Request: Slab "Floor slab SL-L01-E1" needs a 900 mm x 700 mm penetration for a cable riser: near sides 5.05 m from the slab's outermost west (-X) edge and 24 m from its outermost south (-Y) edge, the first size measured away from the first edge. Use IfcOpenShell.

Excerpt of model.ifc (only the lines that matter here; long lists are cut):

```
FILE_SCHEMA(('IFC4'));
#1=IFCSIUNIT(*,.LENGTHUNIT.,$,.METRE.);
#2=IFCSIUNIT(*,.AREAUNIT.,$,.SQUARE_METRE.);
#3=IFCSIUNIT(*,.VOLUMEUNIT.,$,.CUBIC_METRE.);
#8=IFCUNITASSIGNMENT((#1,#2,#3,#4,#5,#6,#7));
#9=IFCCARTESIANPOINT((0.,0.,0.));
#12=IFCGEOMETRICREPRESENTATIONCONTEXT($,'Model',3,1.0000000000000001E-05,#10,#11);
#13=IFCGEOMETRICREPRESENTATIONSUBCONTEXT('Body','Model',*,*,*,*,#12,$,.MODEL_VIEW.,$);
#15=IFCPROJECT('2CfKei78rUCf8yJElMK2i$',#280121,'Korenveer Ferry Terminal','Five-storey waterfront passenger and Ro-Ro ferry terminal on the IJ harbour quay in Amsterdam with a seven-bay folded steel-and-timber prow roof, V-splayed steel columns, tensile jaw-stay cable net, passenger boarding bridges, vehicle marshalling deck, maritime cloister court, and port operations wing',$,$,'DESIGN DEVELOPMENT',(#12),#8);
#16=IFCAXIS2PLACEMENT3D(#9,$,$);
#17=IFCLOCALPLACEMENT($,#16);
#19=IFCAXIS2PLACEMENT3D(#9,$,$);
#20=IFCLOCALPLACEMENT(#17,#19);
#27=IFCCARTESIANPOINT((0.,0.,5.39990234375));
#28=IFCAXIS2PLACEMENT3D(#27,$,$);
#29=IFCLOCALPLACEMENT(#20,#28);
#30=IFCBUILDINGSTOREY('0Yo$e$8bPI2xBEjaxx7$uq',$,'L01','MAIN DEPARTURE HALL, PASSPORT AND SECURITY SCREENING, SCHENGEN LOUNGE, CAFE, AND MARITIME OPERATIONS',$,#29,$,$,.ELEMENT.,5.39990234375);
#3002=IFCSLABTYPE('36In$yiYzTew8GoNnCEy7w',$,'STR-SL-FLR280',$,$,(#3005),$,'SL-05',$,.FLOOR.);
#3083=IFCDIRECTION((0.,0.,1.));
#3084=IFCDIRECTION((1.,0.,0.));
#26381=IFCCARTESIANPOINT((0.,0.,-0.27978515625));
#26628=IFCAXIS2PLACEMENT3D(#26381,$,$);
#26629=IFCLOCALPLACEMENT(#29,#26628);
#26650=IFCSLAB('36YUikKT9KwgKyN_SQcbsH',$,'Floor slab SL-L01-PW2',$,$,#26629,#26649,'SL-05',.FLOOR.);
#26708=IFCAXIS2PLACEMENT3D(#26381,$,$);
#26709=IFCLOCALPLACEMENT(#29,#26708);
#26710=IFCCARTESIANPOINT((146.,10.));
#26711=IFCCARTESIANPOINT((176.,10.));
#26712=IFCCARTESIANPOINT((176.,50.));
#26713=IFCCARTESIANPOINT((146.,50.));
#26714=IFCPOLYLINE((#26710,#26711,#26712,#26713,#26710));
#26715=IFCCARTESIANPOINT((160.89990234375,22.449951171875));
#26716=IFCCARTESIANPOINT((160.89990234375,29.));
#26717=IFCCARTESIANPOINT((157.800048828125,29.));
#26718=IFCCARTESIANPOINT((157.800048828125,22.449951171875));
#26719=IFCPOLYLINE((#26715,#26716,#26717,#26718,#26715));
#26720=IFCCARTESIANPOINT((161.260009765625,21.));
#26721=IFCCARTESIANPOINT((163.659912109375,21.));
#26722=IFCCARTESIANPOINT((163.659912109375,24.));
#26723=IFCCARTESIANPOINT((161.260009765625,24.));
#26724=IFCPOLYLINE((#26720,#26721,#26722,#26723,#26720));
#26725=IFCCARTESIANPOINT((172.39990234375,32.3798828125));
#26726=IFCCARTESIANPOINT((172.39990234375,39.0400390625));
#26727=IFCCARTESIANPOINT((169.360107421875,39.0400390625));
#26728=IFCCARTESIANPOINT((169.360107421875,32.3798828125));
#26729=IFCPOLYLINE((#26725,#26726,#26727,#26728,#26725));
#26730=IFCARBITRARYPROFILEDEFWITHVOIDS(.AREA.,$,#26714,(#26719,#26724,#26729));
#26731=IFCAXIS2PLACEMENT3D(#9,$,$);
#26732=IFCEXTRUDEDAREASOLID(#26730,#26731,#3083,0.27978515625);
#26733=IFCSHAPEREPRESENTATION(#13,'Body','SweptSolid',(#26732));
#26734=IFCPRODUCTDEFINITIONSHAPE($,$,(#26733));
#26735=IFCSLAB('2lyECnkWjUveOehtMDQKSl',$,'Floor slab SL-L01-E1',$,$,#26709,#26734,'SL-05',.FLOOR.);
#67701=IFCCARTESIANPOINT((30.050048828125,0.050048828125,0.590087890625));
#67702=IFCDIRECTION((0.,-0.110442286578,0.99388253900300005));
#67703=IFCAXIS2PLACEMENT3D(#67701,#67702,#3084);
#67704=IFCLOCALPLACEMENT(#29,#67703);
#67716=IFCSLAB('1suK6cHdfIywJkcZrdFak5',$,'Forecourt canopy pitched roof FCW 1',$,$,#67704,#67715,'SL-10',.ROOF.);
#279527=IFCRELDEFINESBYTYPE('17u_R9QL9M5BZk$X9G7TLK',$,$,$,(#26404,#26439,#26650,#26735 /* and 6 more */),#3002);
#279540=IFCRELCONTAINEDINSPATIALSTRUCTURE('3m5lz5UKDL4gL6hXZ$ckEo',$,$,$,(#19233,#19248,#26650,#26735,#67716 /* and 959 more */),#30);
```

```python
import numpy as np
import ifcopenshell
import ifcopenshell.api.feature
import ifcopenshell.api.geometry
import ifcopenshell.api.root
import ifcopenshell.geom
import ifcopenshell.util.placement
import ifcopenshell.util.representation
import ifcopenshell.util.shape
import ifcopenshell.util.unit

model = ifcopenshell.open("model.ifc")
unit_scale = ifcopenshell.util.unit.calculate_unit_scale(model)
settings = ifcopenshell.geom.settings()


def volume(element):
    """Net volume in cubic metres, openings subtracted."""
    shape = ifcopenshell.geom.create_shape(settings, element)
    return ifcopenshell.util.shape.get_volume(shape.geometry)


slab = model.by_guid("2lyECnkWjUveOehtMDQKSl")
before = volume(slab)

# Extent in the slab's own axes, in metres. The edges named are its -X and -Y sides.
slab_shape = ifcopenshell.geom.create_shape(settings, slab)
vertices = ifcopenshell.util.shape.get_vertices(slab_shape.geometry)
x_min, y_min, bottom = vertices.min(axis=0)
top = vertices[:, 2].max()

opening = ifcopenshell.api.root.create_entity(model, ifc_class="IfcOpeningElement", name="Cable riser opening", predefined_type="OPENING")
context = ifcopenshell.util.representation.get_context(model, "Model", "Body", "MODEL_VIEW")
width, depth = 0.9, 0.7
outline = [(0.0, 0.0), (width, 0.0), (width, depth), (0.0, depth), (0.0, 0.0)]
# Overshoot both faces by 50 mm so the cut is clean.
shape = ifcopenshell.api.geometry.add_slab_representation(
    model, context=context, depth=top - bottom + 0.1, polyline=outline
)
ifcopenshell.api.geometry.assign_representation(model, product=opening, representation=shape)

matrix = ifcopenshell.util.placement.get_local_placement(slab.ObjectPlacement)
matrix[:, 3] = matrix @ np.append(np.array([x_min + 5.05, y_min + 24, bottom - 0.05]) / unit_scale, 1.0)
ifcopenshell.api.geometry.edit_object_placement(model, product=opening, matrix=matrix, is_si=False)
ifcopenshell.api.feature.add_feature(model, feature=opening, element=slab)

after = volume(slab)

print(f"slab volume {before:.3f} -> {after:.3f} m3")

model.write("model_edited.ifc")
```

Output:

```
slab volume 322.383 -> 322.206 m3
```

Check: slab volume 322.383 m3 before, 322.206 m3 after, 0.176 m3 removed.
